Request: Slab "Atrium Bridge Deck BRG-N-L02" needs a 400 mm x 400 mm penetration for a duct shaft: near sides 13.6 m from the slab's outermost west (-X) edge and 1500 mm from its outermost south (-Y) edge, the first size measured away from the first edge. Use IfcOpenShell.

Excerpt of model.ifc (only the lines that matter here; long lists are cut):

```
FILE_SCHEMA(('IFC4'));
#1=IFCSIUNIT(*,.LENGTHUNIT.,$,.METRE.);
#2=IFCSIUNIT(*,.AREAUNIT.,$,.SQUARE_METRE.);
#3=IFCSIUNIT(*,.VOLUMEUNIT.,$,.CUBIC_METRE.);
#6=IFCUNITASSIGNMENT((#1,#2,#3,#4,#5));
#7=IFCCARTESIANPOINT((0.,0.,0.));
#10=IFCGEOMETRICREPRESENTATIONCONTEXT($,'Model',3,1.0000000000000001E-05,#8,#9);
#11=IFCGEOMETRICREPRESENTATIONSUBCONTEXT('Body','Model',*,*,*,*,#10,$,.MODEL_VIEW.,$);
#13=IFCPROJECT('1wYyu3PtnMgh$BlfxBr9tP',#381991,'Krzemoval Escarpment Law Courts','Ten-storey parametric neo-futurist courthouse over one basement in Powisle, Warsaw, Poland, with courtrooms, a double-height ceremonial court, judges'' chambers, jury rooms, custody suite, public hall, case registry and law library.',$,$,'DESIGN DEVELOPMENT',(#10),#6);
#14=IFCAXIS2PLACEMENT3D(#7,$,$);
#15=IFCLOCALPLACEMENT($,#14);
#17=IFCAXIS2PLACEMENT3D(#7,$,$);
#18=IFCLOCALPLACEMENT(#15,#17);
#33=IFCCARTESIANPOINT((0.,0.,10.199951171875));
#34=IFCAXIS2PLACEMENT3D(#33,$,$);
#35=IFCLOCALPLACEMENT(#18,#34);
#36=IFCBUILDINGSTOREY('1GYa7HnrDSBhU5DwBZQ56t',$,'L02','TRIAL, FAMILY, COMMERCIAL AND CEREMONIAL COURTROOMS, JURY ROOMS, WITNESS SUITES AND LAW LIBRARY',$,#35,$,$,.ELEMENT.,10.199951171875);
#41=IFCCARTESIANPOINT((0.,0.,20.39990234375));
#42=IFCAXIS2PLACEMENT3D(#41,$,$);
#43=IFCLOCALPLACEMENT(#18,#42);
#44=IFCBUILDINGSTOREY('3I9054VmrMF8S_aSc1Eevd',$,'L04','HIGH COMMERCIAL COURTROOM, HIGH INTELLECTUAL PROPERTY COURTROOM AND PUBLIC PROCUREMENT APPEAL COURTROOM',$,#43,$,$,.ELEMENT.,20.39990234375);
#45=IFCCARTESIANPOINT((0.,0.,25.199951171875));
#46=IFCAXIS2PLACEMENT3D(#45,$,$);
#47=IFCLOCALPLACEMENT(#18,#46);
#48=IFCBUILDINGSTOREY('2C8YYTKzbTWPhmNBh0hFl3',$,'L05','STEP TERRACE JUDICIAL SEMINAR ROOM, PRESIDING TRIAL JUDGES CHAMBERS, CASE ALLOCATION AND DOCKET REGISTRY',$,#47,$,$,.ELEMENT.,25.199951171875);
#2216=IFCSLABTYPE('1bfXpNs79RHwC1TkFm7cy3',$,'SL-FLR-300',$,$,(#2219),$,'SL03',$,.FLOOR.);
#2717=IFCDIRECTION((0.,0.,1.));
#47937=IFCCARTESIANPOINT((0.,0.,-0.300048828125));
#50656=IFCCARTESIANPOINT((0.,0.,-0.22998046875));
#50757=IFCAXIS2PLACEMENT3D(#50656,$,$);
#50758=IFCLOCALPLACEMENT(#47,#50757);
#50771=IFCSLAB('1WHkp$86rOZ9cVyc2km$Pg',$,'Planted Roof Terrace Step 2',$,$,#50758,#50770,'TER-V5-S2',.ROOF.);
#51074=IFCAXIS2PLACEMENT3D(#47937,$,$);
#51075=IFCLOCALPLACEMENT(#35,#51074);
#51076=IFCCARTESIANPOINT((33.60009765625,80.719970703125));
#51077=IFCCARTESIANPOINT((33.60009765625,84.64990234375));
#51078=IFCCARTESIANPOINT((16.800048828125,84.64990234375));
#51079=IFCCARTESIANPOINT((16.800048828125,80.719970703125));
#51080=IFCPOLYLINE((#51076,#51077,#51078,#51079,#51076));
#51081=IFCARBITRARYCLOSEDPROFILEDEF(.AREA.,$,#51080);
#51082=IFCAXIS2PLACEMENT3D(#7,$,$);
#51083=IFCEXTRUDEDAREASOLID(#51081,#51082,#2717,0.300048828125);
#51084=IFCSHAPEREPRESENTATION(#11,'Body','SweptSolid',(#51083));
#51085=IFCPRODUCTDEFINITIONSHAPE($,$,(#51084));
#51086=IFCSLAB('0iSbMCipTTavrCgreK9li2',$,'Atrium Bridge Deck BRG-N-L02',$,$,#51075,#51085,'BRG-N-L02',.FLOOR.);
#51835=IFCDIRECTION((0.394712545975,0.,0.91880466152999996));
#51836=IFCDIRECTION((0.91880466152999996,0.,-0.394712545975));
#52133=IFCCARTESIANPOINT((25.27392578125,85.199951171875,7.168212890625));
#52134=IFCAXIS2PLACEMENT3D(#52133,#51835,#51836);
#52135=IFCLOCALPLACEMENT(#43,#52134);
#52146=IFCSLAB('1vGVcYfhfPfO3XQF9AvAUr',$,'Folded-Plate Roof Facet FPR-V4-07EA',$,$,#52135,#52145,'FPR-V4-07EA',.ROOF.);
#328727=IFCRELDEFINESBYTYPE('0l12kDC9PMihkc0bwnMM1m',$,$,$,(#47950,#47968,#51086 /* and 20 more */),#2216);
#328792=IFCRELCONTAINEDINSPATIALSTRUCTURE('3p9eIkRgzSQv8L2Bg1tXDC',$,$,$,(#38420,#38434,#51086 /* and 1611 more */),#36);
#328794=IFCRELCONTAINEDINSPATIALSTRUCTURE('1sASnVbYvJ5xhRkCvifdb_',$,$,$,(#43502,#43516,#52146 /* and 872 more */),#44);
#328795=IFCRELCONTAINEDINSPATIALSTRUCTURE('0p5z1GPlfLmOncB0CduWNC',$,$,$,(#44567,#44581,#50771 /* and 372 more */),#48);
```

```python
import numpy as np
import ifcopenshell
import ifcopenshell.api.feature
import ifcopenshell.api.geometry
import ifcopenshell.api.root
import ifcopenshell.geom
import ifcopenshell.util.placement
import ifcopenshell.util.representation
import ifcopenshell.util.shape
import ifcopenshell.util.unit

model = ifcopenshell.open("model.ifc")
unit_scale = ifcopenshell.util.unit.calculate_unit_scale(model)
settings = ifcopenshell.geom.settings()


def volume(element):
    """Net volume in cubic metres, openings subtracted."""
    shape = ifcopenshell.geom.create_shape(settings, element)
    return ifcopenshell.util.shape.get_volume(shape.geometry)


slab = model.by_guid("0iSbMCipTTavrCgreK9li2")
before = volume(slab)

# Extent in the slab's own axes, in metres. The edges named are its -X and -Y sides.
slab_shape = ifcopenshell.geom.create_shape(settings, slab)
vertices = ifcopenshell.util.shape.get_vertices(slab_shape.geometry)
x_min, y_min, bottom = vertices.min(axis=0)
top = vertices[:, 2].max()

opening = ifcopenshell.api.root.create_entity(model, ifc_class="IfcOpeningElement", name="Duct shaft opening", predefined_type="OPENING")
context = ifcopenshell.util.representation.get_context(model, "Model", "Body", "MODEL_VIEW")
width, depth = 0.4, 0.4
outline = [(0.0, 0.0), (width, 0.0), (width, depth), (0.0, depth), (0.0, 0.0)]
# Overshoot both faces by 50 mm so the cut is clean.
shape = ifcopenshell.api.geometry.add_slab_representation(
    model, context=context, depth=top - bottom + 0.1, polyline=outline
)
ifcopenshell.api.geometry.assign_representation(model, product=opening, representation=shape)

matrix = ifcopenshell.util.placement.get_local_placement(slab.ObjectPlacement)
matrix[:, 3] = matrix @ np.append(np.array([x_min + 13.6, y_min + 1.5, bottom - 0.05]) / unit_scale, 1.0)
ifcopenshell.api.geometry.edit_object_placement(model, product=opening, matrix=matrix, is_si=False)
ifcopenshell.api.feature.add_feature(model, feature=opening, element=slab)

after = volume(slab)

print(f"slab volume {before:.3f} -> {after:.3f} m3")

model.write("model_rev.ifc")
```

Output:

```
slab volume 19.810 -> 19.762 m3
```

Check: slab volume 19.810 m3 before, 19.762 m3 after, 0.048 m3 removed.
